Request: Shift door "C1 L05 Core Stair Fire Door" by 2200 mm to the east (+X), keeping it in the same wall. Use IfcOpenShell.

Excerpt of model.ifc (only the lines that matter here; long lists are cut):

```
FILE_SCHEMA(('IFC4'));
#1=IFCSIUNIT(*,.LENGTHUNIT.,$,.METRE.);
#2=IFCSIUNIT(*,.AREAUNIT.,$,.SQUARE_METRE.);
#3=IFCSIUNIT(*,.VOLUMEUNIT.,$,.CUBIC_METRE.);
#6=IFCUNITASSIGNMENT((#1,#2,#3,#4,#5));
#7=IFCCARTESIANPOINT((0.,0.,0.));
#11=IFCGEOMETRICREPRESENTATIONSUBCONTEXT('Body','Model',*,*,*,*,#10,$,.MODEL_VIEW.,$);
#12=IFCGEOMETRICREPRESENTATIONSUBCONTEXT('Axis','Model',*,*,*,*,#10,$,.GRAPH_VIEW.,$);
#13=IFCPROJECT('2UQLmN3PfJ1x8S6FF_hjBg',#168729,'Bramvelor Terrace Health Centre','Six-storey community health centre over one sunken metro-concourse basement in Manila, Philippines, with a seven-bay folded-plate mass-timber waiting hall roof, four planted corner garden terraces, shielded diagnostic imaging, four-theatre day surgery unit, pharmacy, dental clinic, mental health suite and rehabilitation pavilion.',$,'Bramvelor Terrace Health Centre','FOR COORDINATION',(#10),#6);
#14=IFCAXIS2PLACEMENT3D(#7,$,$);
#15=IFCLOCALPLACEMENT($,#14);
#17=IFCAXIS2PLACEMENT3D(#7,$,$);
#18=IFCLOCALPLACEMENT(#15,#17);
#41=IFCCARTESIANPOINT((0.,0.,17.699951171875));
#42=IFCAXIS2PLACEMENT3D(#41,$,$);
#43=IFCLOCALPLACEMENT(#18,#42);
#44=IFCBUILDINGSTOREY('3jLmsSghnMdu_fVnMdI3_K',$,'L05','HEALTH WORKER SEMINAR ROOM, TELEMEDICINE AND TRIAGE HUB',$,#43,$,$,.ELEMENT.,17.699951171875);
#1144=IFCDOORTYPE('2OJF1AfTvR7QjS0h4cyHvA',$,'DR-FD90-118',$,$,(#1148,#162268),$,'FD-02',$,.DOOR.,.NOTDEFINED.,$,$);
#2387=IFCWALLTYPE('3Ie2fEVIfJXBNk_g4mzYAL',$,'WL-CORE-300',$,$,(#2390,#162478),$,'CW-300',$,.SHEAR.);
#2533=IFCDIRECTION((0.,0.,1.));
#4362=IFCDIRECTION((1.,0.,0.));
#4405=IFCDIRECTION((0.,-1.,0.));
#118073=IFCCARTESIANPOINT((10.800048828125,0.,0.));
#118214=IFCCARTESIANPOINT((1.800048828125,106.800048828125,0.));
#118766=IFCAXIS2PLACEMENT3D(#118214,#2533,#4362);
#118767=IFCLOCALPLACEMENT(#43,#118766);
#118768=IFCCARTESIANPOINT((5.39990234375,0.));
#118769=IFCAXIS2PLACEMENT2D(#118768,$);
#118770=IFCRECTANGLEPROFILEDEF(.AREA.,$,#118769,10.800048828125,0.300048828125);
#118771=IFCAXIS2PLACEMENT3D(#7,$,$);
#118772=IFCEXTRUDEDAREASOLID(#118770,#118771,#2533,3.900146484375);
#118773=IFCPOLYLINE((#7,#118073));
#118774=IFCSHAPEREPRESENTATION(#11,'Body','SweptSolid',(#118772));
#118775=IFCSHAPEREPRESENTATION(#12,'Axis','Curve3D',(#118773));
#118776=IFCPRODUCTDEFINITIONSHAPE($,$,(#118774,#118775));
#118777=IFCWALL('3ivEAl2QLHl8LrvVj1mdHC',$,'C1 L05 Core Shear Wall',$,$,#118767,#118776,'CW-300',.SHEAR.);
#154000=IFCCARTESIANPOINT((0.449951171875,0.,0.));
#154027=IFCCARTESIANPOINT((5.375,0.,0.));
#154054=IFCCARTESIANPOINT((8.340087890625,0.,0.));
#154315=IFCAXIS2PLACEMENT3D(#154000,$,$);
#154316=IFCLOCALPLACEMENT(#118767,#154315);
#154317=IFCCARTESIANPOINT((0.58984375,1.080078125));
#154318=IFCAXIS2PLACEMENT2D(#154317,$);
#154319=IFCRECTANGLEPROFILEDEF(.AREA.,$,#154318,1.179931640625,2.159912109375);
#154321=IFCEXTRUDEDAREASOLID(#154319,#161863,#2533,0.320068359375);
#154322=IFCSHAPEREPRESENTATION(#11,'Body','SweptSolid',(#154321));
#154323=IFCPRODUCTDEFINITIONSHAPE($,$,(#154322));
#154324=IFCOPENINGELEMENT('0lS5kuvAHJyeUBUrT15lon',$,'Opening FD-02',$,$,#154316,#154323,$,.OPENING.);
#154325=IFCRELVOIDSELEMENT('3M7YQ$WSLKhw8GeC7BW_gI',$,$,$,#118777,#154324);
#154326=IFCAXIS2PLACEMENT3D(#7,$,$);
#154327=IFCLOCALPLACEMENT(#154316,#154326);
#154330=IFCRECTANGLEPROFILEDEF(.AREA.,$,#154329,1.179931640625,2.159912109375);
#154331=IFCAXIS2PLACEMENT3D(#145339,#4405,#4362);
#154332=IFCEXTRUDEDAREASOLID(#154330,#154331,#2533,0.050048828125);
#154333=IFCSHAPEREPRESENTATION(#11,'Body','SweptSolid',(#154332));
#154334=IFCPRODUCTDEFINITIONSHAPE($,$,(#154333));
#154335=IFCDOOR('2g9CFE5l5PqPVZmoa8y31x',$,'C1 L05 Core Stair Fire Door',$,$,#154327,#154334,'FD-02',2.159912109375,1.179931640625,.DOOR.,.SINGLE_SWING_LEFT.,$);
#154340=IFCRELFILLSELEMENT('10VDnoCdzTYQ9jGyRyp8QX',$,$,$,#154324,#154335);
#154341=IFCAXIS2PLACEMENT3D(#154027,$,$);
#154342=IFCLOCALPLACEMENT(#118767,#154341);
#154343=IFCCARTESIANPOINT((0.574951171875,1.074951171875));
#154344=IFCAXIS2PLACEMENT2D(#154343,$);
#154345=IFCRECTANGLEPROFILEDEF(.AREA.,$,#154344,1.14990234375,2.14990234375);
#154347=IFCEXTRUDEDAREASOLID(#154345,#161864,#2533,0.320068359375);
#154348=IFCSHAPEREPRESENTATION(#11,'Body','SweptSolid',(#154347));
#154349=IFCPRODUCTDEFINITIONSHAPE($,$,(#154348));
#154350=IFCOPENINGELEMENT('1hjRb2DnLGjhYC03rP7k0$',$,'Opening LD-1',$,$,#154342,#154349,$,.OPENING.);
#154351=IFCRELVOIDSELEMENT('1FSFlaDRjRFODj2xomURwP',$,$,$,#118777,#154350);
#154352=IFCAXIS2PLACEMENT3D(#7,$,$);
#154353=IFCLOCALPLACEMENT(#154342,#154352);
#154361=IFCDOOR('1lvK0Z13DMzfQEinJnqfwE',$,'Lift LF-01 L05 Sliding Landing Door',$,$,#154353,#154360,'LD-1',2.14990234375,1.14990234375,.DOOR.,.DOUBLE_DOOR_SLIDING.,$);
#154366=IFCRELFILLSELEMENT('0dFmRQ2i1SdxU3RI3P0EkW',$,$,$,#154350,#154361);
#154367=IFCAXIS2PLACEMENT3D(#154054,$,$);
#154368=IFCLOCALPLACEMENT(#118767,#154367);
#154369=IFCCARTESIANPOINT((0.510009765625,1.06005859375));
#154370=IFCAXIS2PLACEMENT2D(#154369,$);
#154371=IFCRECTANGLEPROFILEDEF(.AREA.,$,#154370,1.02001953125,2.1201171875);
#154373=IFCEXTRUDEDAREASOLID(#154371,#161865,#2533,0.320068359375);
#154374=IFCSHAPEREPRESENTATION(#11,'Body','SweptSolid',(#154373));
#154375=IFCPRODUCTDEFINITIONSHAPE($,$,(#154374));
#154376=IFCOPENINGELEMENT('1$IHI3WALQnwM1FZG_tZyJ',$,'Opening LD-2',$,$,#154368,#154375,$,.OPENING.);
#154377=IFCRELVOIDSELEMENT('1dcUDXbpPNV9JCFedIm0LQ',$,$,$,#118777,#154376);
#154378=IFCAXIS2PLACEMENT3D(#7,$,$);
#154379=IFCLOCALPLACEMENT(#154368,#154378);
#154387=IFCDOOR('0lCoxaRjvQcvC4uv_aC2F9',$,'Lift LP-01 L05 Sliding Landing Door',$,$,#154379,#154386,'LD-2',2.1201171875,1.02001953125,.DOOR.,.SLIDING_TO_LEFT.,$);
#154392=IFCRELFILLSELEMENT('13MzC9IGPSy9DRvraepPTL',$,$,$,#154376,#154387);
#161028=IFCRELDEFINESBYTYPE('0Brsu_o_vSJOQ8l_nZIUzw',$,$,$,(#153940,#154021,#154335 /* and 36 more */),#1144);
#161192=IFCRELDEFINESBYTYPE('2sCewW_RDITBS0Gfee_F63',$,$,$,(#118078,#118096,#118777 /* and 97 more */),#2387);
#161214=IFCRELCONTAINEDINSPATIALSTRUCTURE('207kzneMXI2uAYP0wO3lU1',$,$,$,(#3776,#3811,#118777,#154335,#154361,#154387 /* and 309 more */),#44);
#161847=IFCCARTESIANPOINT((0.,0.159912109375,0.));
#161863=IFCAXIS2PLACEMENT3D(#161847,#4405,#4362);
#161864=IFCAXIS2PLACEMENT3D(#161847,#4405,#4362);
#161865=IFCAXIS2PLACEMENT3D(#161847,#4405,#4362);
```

```python
import ifcopenshell
import ifcopenshell.api.geometry
import ifcopenshell.util.placement

model = ifcopenshell.open("model.ifc")

door = model.by_id(154335)
opening = door.FillsVoids[0].RelatingOpeningElement
wall = opening.VoidsElements[0].RelatingBuildingElement

wall_matrix = ifcopenshell.util.placement.get_local_placement(wall.ObjectPlacement)
shift = wall_matrix[:3, 0] * 2.2
before = ifcopenshell.util.placement.get_local_placement(door.ObjectPlacement)[:3, 3].copy()

# The door is placed relative to its opening, so it follows when the opening moves.
matrix = ifcopenshell.util.placement.get_local_placement(opening.ObjectPlacement)
matrix[:3, 3] += shift
ifcopenshell.api.geometry.edit_object_placement(
    model, product=opening, matrix=matrix, is_si=False, should_transform_children=True
)

after = ifcopenshell.util.placement.get_local_placement(door.ObjectPlacement)[:3, 3]
print("door moved by", (after - before).round(3) + 0.0)

model.write("model_rev.ifc")
```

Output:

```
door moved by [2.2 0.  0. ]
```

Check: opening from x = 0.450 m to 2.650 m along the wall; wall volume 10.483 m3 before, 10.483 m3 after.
